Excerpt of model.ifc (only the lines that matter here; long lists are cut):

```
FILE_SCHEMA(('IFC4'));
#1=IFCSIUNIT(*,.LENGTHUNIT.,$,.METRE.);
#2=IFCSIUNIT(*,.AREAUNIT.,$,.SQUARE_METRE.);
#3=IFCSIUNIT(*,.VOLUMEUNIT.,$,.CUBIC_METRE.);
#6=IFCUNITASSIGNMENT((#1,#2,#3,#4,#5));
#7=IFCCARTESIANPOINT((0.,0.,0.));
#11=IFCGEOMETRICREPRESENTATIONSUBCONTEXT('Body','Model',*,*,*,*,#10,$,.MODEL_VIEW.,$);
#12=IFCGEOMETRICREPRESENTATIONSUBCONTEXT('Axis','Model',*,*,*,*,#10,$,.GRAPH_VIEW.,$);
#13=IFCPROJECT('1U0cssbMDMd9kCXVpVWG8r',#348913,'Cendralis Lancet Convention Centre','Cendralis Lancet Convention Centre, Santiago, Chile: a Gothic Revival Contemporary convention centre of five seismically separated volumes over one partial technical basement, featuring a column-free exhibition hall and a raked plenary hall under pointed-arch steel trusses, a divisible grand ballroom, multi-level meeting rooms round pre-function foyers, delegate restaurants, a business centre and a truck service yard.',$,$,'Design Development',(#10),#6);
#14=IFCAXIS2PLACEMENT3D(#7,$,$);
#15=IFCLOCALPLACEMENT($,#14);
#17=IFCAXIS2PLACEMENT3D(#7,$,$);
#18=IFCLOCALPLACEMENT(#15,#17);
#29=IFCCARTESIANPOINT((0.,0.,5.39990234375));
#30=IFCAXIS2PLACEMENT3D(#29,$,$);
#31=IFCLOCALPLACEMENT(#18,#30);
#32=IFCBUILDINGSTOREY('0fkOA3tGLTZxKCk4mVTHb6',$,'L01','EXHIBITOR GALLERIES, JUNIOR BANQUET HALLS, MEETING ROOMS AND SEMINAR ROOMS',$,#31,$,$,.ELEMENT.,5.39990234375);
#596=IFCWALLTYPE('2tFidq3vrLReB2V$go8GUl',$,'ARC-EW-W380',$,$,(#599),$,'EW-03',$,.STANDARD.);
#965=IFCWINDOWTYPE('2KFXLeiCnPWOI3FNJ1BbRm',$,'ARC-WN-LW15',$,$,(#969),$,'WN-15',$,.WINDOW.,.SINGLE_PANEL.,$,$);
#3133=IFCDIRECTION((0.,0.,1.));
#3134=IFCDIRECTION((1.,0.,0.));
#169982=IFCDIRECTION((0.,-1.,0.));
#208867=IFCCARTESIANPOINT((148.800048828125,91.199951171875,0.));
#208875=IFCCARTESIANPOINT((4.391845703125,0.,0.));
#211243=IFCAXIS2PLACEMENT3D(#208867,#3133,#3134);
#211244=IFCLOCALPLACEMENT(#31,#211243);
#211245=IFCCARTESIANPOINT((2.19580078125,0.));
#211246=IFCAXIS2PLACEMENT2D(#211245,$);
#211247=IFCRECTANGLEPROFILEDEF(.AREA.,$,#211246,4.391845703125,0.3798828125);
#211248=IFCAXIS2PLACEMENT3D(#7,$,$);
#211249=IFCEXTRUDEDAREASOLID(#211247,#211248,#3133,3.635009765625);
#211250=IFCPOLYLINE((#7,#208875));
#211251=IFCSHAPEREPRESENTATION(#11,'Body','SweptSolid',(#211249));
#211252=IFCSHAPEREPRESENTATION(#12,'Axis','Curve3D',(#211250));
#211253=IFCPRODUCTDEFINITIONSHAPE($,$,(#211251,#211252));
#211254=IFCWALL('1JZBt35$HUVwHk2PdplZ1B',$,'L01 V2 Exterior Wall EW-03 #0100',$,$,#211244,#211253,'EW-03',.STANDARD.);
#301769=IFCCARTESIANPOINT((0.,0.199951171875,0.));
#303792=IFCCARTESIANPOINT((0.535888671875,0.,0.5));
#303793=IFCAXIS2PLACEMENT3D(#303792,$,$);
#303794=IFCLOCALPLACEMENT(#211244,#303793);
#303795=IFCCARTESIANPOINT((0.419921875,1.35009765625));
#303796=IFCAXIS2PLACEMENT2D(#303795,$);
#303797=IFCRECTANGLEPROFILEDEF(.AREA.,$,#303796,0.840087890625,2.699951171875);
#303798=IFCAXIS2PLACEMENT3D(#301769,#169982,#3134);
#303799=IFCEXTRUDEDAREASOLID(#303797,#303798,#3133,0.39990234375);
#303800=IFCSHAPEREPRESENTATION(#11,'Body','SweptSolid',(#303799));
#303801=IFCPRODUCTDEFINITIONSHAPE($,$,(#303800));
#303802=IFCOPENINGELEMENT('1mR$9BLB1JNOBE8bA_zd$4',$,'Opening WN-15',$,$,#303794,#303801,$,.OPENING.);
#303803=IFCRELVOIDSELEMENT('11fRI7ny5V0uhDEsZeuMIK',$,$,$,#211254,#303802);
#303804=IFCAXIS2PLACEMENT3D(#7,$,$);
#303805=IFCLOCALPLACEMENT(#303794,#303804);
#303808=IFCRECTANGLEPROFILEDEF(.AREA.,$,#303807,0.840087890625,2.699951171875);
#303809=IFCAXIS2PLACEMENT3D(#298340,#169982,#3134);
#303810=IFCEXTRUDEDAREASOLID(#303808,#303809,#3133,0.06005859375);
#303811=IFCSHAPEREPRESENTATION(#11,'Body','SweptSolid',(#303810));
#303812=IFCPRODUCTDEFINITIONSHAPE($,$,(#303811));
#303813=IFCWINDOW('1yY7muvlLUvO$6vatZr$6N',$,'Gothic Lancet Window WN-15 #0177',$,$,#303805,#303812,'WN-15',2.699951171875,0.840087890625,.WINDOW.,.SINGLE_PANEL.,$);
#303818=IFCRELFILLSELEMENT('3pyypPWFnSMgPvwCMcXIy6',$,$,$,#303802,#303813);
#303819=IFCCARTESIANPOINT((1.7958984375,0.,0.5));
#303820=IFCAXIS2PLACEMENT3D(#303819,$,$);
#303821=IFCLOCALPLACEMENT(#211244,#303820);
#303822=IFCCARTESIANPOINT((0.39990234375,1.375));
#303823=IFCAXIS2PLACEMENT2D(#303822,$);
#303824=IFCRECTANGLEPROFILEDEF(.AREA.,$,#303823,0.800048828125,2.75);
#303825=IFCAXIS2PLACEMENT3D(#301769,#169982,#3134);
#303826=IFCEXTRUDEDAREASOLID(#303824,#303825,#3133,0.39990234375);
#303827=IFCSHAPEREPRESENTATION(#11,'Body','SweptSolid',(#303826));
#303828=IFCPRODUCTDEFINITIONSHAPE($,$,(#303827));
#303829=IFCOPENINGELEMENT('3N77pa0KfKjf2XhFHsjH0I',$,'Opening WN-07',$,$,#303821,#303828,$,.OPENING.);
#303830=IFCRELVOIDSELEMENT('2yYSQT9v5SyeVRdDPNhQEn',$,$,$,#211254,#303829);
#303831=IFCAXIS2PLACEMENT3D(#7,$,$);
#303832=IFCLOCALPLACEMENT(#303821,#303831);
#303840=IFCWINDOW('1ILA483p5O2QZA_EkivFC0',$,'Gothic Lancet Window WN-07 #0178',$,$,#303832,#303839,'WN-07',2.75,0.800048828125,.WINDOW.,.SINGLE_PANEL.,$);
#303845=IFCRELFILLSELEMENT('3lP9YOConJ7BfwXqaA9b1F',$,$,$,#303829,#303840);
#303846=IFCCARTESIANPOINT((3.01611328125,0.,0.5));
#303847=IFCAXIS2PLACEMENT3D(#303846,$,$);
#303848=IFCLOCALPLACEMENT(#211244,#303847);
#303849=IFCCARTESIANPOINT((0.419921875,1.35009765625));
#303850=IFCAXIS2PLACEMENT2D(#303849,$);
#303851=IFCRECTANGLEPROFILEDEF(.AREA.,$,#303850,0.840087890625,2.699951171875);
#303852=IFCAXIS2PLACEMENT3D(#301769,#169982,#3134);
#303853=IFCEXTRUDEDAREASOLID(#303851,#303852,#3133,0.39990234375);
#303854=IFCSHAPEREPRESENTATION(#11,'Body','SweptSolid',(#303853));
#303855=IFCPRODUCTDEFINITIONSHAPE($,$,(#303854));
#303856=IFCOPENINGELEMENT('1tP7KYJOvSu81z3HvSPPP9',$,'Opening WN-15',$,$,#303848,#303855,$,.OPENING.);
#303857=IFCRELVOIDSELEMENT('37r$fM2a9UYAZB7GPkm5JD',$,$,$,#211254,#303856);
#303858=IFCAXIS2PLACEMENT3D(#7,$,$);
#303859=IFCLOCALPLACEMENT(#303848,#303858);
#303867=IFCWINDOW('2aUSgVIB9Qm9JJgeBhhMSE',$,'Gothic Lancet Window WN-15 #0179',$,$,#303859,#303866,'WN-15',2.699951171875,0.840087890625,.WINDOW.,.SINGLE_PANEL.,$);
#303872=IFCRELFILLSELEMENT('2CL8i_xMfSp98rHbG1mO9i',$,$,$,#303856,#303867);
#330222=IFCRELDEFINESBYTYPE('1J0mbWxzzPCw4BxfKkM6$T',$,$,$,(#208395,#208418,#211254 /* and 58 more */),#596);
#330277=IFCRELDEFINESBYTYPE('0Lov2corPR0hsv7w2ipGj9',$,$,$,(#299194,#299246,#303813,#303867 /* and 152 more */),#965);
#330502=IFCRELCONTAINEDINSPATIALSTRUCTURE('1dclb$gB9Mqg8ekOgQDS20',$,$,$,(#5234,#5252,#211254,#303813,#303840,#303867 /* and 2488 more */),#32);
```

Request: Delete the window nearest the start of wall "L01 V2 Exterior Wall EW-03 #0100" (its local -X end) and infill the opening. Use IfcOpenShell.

```python
import ifcopenshell
import ifcopenshell.api.feature
import ifcopenshell.api.root
import ifcopenshell.geom
import ifcopenshell.util.shape

model = ifcopenshell.open("model.ifc")
settings = ifcopenshell.geom.settings()


def volume(element):
    """Net volume in cubic metres, openings subtracted."""
    shape = ifcopenshell.geom.create_shape(settings, element)
    return ifcopenshell.util.shape.get_volume(shape.geometry)


window = model.by_guid("1yY7muvlLUvO$6vatZr$6N")
opening = window.FillsVoids[0].RelatingOpeningElement
wall = opening.VoidsElements[0].RelatingBuildingElement
before = volume(wall)

ifcopenshell.api.root.remove_product(model, product=window)
ifcopenshell.api.feature.remove_feature(model, feature=opening)

after = volume(wall)

print(f"wall volume {before:.3f} -> {after:.3f} m3")

model.write("model_rev.ifc")
```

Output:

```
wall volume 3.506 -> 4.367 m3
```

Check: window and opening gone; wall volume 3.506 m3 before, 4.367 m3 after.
